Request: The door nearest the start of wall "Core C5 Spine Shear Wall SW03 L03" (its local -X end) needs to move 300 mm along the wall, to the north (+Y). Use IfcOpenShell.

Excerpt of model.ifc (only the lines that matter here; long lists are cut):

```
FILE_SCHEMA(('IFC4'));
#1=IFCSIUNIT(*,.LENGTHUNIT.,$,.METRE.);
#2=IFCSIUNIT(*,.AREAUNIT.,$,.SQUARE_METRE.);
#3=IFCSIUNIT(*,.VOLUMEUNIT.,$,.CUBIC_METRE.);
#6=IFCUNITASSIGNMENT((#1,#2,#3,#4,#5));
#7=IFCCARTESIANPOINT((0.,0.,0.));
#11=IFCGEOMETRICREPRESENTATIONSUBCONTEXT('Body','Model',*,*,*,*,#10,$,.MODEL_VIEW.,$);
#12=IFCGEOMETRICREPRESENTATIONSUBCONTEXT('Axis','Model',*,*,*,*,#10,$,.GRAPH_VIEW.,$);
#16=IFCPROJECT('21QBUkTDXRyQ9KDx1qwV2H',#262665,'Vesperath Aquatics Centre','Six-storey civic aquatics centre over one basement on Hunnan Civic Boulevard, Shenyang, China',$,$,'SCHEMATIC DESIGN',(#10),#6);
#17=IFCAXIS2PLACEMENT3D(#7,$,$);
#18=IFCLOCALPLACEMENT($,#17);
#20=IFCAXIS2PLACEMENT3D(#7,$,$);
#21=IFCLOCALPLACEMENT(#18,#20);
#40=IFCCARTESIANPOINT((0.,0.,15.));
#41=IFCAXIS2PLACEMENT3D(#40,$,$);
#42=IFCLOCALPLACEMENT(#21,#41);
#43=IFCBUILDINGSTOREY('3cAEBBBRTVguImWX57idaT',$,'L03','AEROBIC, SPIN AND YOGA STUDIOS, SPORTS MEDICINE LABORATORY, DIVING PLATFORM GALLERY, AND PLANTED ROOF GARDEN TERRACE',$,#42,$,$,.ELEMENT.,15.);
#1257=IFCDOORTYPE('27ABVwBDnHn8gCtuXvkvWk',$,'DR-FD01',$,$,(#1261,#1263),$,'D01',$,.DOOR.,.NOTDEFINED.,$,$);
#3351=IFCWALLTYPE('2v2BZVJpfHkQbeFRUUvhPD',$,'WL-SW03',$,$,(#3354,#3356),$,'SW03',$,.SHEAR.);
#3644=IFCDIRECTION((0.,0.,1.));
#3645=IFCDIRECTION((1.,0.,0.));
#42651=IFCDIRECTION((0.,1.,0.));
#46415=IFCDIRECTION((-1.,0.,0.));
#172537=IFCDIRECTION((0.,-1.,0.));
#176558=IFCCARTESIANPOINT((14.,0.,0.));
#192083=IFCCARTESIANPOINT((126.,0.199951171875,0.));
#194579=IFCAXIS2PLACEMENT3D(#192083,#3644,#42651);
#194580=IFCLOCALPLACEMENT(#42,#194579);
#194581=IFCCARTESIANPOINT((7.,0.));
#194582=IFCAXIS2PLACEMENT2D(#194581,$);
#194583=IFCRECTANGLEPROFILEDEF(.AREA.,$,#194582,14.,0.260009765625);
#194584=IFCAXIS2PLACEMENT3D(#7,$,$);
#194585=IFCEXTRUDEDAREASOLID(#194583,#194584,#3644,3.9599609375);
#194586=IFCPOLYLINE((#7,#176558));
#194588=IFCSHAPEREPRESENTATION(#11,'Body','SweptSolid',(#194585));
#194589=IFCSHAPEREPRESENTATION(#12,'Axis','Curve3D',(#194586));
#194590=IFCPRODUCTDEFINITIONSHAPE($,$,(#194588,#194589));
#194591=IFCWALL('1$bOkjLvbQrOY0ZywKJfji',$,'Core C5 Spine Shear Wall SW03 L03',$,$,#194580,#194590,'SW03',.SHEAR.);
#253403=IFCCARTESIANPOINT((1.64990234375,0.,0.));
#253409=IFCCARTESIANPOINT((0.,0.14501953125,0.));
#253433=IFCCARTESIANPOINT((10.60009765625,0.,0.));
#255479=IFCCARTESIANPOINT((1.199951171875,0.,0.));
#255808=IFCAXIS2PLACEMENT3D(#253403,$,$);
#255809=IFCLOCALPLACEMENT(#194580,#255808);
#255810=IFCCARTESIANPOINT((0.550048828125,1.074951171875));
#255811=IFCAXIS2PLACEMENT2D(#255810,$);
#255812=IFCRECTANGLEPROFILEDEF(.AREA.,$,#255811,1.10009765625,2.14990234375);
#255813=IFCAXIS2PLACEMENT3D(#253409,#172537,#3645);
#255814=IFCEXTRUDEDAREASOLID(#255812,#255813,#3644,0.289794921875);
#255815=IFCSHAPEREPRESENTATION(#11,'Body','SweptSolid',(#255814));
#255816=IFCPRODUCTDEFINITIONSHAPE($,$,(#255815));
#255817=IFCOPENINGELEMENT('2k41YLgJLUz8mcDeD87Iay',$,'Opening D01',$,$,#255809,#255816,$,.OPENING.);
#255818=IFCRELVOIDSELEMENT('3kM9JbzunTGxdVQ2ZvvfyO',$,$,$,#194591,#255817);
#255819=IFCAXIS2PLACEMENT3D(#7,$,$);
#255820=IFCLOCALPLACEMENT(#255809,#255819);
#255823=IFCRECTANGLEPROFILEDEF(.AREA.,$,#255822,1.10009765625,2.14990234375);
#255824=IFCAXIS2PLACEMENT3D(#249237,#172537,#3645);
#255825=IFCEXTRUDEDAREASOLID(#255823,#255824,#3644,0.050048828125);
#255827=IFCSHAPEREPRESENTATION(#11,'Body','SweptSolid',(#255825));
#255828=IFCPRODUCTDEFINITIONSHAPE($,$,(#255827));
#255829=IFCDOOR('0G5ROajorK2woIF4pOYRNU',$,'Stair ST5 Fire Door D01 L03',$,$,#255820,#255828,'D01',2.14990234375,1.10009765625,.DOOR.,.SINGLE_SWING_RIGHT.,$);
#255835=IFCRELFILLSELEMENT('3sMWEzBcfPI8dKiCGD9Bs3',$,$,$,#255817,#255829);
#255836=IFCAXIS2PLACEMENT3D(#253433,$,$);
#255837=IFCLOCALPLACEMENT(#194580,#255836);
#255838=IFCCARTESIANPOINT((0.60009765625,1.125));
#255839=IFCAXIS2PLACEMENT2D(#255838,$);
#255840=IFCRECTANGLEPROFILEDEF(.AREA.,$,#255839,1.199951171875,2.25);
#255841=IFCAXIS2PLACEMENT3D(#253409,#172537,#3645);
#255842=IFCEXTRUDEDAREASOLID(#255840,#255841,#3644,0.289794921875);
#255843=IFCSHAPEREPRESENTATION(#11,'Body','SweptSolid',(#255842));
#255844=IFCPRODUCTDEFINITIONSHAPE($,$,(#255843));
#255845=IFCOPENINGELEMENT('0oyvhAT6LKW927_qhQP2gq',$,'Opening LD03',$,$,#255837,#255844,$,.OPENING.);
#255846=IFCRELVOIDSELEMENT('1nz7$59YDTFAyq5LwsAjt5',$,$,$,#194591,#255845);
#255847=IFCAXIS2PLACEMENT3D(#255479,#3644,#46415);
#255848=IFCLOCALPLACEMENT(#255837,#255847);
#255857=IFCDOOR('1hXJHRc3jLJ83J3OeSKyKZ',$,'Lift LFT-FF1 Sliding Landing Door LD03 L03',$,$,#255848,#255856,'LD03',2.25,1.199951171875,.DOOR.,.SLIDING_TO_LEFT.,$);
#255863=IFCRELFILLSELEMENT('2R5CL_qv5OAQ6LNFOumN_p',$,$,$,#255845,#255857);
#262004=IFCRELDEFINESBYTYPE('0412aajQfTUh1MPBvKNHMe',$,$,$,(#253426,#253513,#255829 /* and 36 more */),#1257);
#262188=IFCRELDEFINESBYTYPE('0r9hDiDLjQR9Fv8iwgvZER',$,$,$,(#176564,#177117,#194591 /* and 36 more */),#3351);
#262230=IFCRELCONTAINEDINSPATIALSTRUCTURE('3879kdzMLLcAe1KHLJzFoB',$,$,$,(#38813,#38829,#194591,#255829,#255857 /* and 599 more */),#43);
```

```python
import ifcopenshell
import ifcopenshell.api.geometry
import ifcopenshell.util.placement

model = ifcopenshell.open("model.ifc")

door = model.by_guid("0G5ROajorK2woIF4pOYRNU")
opening = door.FillsVoids[0].RelatingOpeningElement
wall = opening.VoidsElements[0].RelatingBuildingElement

wall_matrix = ifcopenshell.util.placement.get_local_placement(wall.ObjectPlacement)
shift = wall_matrix[:3, 0] * 0.3
before = ifcopenshell.util.placement.get_local_placement(door.ObjectPlacement)[:3, 3].copy()

# The door is placed relative to its opening, so it follows when the opening moves.
matrix = ifcopenshell.util.placement.get_local_placement(opening.ObjectPlacement)
matrix[:3, 3] += shift
ifcopenshell.api.geometry.edit_object_placement(
    model, product=opening, matrix=matrix, is_si=False, should_transform_children=True
)

after = ifcopenshell.util.placement.get_local_placement(door.ObjectPlacement)[:3, 3]
print("door moved by", (after - before).round(3) + 0.0)

model.write("model_edited.ifc")
```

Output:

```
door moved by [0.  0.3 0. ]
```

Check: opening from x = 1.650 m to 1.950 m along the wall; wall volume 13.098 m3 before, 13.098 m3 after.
